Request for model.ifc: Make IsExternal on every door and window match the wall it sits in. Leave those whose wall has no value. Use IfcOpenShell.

First a look at what the model holds.

```python
import ifcopenshell
import ifcopenshell.util.element

model = ifcopenshell.open("model.ifc")
print(model.schema)
seen = {}
for e in model.by_type("IfcDoor") + model.by_type("IfcWindow"):
    if not e.FillsVoids:
        continue
    host = e.FillsVoids[0].RelatingOpeningElement.VoidsElements[0].RelatingBuildingElement
    own = ifcopenshell.util.element.get_pset(e, f"Pset_{e.is_a()[3:].removesuffix('StandardCase')}Common", "IsExternal")
    wall = ifcopenshell.util.element.get_pset(host, "Pset_WallCommon", "IsExternal")
    seen[e.is_a(), own, wall] = seen.get((e.is_a(), own, wall), 0) + 1
for (cls, own, wall), count in sorted(seen.items(), key=str):
    print(count, cls, "IsExternal:", own, "| host wall:", wall)
```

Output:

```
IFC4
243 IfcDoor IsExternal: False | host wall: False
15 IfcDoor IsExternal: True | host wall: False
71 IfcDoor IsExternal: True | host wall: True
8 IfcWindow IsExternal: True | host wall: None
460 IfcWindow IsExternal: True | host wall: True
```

```python
import ifcopenshell
import ifcopenshell.api.pset
import ifcopenshell.util.element

model = ifcopenshell.open("model.ifc")

count = 0
for ifc_class, pset_name in (("IfcDoor", "Pset_DoorCommon"), ("IfcWindow", "Pset_WindowCommon")):
    for e in model.by_type(ifc_class):
        if not e.FillsVoids:
            continue
        host = e.FillsVoids[0].RelatingOpeningElement.VoidsElements[0].RelatingBuildingElement
        external = ifcopenshell.util.element.get_pset(host, "Pset_WallCommon", "IsExternal")
        if external is None or ifcopenshell.util.element.get_pset(e, pset_name, "IsExternal") == external:
            continue
        pset = ifcopenshell.api.pset.add_pset(model, product=e, name=pset_name)
        ifcopenshell.api.pset.edit_pset(model, pset=pset, properties={"IsExternal": external})
        count += 1

print(count, "updated")

model.write("model-out.ifc")
```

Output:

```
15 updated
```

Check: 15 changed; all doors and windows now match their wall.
